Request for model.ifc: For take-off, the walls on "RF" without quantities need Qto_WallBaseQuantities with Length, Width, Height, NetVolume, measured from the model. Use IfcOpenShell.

First a look at what the model holds.

```python
import ifcopenshell
import ifcopenshell.util.element
import ifcopenshell.util.unit

model = ifcopenshell.open("model.ifc")
print(model.schema)
for unit_type in ("LENGTHUNIT", "AREAUNIT", "VOLUMEUNIT"):
    print(unit_type, ifcopenshell.util.unit.calculate_unit_scale(model, unit_type))
storey = next(s for s in model.by_type("IfcBuildingStorey") if s.Name == "RF")
walls = [e for e in ifcopenshell.util.element.get_decomposition(storey) if e.is_a("IfcWall")]
for e in sorted(walls, key=lambda e: e.id()):
    print(e.id(), e.is_a(), e.Name, list(ifcopenshell.util.element.get_psets(e, qtos_only=True)), sep=" | ")
```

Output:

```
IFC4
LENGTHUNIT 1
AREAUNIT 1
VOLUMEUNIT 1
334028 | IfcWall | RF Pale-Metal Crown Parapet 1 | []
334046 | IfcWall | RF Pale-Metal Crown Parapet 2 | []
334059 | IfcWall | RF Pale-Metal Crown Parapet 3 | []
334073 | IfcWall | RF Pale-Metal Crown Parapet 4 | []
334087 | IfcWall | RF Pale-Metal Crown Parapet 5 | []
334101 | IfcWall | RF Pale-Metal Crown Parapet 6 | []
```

```python
import ifcopenshell
import ifcopenshell.api.pset
import ifcopenshell.geom
import ifcopenshell.util.element
import ifcopenshell.util.shape
import ifcopenshell.util.unit

model = ifcopenshell.open("model.ifc")
unit_scale = ifcopenshell.util.unit.calculate_unit_scale(model)
volume_scale = ifcopenshell.util.unit.calculate_unit_scale(model, "VOLUMEUNIT")
settings = ifcopenshell.geom.settings()

storey = next(s for s in model.by_type("IfcBuildingStorey") if s.Name == "RF")
walls = [e for e in ifcopenshell.util.element.get_decomposition(storey) if e.is_a("IfcWall")]

for e in sorted(walls, key=lambda e: e.id()):
    if ifcopenshell.util.element.get_psets(e, qtos_only=True, should_inherit=False):
        continue
    # Geometry comes back in metres, in the element's own axes.
    shape = ifcopenshell.geom.create_shape(settings, e)
    values = {
        "Length": ifcopenshell.util.shape.get_x(shape.geometry) / unit_scale,
        "Width": ifcopenshell.util.shape.get_y(shape.geometry) / unit_scale,
        "Height": ifcopenshell.util.shape.get_z(shape.geometry) / unit_scale,
        "NetVolume": ifcopenshell.util.shape.get_volume(shape.geometry) / volume_scale,
    }
    qto = ifcopenshell.api.pset.add_qto(model, product=e, name="Qto_WallBaseQuantities")
    ifcopenshell.api.pset.edit_qto(model, qto=qto, properties=values)
    print(e.id(), {k: round(v, 3) for k, v in values.items()})

model.write("model_updated.ifc")
```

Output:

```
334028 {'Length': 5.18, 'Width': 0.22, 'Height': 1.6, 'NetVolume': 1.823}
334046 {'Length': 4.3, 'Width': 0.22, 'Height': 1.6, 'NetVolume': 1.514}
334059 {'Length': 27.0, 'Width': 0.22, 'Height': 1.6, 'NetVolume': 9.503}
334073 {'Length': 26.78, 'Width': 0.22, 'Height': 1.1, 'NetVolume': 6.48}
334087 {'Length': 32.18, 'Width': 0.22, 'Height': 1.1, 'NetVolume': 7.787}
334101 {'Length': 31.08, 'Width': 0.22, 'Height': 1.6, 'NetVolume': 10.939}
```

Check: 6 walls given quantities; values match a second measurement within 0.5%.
